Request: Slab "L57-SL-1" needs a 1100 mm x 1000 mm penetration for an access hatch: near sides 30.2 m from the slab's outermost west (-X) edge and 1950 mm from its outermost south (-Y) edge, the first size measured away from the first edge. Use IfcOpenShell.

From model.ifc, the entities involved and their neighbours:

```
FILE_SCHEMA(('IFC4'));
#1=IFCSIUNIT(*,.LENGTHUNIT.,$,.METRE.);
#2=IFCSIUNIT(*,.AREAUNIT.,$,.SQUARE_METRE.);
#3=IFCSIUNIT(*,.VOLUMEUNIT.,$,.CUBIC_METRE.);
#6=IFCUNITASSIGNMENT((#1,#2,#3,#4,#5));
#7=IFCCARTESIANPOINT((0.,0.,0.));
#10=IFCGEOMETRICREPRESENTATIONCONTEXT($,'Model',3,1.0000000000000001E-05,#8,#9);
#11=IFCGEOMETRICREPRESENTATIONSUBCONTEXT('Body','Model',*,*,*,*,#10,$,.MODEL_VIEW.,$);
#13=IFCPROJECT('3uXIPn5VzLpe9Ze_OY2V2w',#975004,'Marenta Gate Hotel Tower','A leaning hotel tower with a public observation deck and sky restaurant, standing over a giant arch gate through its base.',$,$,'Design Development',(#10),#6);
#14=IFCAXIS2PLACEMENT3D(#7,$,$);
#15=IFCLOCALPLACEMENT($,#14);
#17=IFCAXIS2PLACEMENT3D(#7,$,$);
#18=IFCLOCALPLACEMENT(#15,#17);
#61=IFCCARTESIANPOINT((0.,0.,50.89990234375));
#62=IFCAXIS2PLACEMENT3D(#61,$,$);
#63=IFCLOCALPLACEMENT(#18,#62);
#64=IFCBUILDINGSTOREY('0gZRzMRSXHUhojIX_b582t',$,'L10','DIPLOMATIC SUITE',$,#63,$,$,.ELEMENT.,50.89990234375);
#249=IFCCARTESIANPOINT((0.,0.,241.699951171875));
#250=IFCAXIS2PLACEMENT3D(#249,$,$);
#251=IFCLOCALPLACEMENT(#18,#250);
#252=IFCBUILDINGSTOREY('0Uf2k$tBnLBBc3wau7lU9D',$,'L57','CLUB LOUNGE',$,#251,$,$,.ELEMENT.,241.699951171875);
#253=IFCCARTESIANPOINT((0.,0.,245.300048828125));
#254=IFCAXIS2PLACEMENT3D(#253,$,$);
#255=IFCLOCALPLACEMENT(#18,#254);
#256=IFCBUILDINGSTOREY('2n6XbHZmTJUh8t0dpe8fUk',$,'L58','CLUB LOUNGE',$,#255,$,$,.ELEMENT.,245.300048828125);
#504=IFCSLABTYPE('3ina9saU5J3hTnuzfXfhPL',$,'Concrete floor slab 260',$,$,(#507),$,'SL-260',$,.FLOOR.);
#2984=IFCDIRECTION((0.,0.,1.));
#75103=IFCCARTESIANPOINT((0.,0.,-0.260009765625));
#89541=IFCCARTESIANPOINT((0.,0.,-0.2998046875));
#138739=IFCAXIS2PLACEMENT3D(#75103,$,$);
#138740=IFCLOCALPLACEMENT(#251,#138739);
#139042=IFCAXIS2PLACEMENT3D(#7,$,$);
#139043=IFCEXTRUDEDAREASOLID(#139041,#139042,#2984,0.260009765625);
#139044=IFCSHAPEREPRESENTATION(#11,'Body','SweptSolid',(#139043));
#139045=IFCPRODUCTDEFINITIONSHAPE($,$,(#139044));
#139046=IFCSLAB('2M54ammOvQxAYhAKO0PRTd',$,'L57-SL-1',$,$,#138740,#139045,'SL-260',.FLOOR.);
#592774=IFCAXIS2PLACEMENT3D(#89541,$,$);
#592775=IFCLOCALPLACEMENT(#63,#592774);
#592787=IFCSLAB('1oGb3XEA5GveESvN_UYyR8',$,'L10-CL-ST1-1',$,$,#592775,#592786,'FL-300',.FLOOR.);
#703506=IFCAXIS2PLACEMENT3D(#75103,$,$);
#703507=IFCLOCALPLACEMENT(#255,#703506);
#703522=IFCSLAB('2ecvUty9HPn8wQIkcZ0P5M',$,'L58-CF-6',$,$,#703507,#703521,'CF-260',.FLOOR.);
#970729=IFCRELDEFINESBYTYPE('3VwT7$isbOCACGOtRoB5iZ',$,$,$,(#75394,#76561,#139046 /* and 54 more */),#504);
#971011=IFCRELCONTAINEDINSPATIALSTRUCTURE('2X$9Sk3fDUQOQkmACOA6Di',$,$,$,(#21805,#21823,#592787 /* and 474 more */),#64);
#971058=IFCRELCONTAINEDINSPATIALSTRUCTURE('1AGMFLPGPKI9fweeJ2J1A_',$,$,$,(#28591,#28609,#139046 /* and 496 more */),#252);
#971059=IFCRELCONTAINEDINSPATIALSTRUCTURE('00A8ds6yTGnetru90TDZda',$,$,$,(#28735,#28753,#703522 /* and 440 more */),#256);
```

```python
import numpy as np
import ifcopenshell
import ifcopenshell.api.feature
import ifcopenshell.api.geometry
import ifcopenshell.api.root
import ifcopenshell.geom
import ifcopenshell.util.placement
import ifcopenshell.util.representation
import ifcopenshell.util.shape
import ifcopenshell.util.unit

model = ifcopenshell.open("model.ifc")
unit_scale = ifcopenshell.util.unit.calculate_unit_scale(model)
settings = ifcopenshell.geom.settings()


def volume(element):
    """Net volume in cubic metres, openings subtracted."""
    shape = ifcopenshell.geom.create_shape(settings, element)
    return ifcopenshell.util.shape.get_volume(shape.geometry)


slab = model.by_id(139046)
before = volume(slab)

# Extent in the slab's own axes, in metres. The edges named are its -X and -Y sides.
slab_shape = ifcopenshell.geom.create_shape(settings, slab)
vertices = ifcopenshell.util.shape.get_vertices(slab_shape.geometry)
x_min, y_min, bottom = vertices.min(axis=0)
top = vertices[:, 2].max()

opening = ifcopenshell.api.root.create_entity(model, ifc_class="IfcOpeningElement", name="Access hatch opening", predefined_type="OPENING")
context = ifcopenshell.util.representation.get_context(model, "Model", "Body", "MODEL_VIEW")
width, depth = 1.1, 1
outline = [(0.0, 0.0), (width, 0.0), (width, depth), (0.0, depth), (0.0, 0.0)]
# Overshoot both faces by 50 mm so the cut is clean.
shape = ifcopenshell.api.geometry.add_slab_representation(
    model, context=context, depth=top - bottom + 0.1, polyline=outline
)
ifcopenshell.api.geometry.assign_representation(model, product=opening, representation=shape)

matrix = ifcopenshell.util.placement.get_local_placement(slab.ObjectPlacement)
matrix[:, 3] = matrix @ np.append(np.array([x_min + 30.2, y_min + 1.95, bottom - 0.05]) / unit_scale, 1.0)
ifcopenshell.api.geometry.edit_object_placement(model, product=opening, matrix=matrix, is_si=False)
ifcopenshell.api.feature.add_feature(model, feature=opening, element=slab)

after = volume(slab)

print(f"slab volume {before:.3f} -> {after:.3f} m3")

model.write("model_updated.ifc")
```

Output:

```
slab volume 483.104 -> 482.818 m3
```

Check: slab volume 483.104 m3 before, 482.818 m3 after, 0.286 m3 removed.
